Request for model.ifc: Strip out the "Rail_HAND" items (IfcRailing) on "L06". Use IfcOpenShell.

First a look at what the model holds.

```python
import ifcopenshell
import ifcopenshell.util.element

model = ifcopenshell.open("model.ifc")
print(model.schema)
storey = next(s for s in model.by_type("IfcBuildingStorey") if s.Name == "L06")
railings = [e for e in ifcopenshell.util.element.get_decomposition(storey) if e.is_a("IfcRailing")]
seen = {}
for e in railings:
    element_type = ifcopenshell.util.element.get_type(e)
    name = element_type.Name if element_type not in (None, e) else None
    seen[name] = seen.get(name, 0) + 1
for name, count in sorted(seen.items(), key=str):
    print(count, "x", name)
```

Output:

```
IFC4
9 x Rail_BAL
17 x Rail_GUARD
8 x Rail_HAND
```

```python
import ifcopenshell
import ifcopenshell.api.root
import ifcopenshell.util.element

model = ifcopenshell.open("model.ifc")

storey = next(s for s in model.by_type("IfcBuildingStorey") if s.Name == "L06")
railings = [e for e in ifcopenshell.util.element.get_decomposition(storey) if e.is_a("IfcRailing")]
targets = [e for e in railings if (t := ifcopenshell.util.element.get_type(e)) not in (None, e) and t.Name == "Rail_HAND"]

for e in targets:
    ifcopenshell.api.root.remove_product(model, product=e)
print(len(targets), "removed")

model.write("model_rev.ifc")
```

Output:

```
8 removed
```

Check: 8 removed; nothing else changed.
